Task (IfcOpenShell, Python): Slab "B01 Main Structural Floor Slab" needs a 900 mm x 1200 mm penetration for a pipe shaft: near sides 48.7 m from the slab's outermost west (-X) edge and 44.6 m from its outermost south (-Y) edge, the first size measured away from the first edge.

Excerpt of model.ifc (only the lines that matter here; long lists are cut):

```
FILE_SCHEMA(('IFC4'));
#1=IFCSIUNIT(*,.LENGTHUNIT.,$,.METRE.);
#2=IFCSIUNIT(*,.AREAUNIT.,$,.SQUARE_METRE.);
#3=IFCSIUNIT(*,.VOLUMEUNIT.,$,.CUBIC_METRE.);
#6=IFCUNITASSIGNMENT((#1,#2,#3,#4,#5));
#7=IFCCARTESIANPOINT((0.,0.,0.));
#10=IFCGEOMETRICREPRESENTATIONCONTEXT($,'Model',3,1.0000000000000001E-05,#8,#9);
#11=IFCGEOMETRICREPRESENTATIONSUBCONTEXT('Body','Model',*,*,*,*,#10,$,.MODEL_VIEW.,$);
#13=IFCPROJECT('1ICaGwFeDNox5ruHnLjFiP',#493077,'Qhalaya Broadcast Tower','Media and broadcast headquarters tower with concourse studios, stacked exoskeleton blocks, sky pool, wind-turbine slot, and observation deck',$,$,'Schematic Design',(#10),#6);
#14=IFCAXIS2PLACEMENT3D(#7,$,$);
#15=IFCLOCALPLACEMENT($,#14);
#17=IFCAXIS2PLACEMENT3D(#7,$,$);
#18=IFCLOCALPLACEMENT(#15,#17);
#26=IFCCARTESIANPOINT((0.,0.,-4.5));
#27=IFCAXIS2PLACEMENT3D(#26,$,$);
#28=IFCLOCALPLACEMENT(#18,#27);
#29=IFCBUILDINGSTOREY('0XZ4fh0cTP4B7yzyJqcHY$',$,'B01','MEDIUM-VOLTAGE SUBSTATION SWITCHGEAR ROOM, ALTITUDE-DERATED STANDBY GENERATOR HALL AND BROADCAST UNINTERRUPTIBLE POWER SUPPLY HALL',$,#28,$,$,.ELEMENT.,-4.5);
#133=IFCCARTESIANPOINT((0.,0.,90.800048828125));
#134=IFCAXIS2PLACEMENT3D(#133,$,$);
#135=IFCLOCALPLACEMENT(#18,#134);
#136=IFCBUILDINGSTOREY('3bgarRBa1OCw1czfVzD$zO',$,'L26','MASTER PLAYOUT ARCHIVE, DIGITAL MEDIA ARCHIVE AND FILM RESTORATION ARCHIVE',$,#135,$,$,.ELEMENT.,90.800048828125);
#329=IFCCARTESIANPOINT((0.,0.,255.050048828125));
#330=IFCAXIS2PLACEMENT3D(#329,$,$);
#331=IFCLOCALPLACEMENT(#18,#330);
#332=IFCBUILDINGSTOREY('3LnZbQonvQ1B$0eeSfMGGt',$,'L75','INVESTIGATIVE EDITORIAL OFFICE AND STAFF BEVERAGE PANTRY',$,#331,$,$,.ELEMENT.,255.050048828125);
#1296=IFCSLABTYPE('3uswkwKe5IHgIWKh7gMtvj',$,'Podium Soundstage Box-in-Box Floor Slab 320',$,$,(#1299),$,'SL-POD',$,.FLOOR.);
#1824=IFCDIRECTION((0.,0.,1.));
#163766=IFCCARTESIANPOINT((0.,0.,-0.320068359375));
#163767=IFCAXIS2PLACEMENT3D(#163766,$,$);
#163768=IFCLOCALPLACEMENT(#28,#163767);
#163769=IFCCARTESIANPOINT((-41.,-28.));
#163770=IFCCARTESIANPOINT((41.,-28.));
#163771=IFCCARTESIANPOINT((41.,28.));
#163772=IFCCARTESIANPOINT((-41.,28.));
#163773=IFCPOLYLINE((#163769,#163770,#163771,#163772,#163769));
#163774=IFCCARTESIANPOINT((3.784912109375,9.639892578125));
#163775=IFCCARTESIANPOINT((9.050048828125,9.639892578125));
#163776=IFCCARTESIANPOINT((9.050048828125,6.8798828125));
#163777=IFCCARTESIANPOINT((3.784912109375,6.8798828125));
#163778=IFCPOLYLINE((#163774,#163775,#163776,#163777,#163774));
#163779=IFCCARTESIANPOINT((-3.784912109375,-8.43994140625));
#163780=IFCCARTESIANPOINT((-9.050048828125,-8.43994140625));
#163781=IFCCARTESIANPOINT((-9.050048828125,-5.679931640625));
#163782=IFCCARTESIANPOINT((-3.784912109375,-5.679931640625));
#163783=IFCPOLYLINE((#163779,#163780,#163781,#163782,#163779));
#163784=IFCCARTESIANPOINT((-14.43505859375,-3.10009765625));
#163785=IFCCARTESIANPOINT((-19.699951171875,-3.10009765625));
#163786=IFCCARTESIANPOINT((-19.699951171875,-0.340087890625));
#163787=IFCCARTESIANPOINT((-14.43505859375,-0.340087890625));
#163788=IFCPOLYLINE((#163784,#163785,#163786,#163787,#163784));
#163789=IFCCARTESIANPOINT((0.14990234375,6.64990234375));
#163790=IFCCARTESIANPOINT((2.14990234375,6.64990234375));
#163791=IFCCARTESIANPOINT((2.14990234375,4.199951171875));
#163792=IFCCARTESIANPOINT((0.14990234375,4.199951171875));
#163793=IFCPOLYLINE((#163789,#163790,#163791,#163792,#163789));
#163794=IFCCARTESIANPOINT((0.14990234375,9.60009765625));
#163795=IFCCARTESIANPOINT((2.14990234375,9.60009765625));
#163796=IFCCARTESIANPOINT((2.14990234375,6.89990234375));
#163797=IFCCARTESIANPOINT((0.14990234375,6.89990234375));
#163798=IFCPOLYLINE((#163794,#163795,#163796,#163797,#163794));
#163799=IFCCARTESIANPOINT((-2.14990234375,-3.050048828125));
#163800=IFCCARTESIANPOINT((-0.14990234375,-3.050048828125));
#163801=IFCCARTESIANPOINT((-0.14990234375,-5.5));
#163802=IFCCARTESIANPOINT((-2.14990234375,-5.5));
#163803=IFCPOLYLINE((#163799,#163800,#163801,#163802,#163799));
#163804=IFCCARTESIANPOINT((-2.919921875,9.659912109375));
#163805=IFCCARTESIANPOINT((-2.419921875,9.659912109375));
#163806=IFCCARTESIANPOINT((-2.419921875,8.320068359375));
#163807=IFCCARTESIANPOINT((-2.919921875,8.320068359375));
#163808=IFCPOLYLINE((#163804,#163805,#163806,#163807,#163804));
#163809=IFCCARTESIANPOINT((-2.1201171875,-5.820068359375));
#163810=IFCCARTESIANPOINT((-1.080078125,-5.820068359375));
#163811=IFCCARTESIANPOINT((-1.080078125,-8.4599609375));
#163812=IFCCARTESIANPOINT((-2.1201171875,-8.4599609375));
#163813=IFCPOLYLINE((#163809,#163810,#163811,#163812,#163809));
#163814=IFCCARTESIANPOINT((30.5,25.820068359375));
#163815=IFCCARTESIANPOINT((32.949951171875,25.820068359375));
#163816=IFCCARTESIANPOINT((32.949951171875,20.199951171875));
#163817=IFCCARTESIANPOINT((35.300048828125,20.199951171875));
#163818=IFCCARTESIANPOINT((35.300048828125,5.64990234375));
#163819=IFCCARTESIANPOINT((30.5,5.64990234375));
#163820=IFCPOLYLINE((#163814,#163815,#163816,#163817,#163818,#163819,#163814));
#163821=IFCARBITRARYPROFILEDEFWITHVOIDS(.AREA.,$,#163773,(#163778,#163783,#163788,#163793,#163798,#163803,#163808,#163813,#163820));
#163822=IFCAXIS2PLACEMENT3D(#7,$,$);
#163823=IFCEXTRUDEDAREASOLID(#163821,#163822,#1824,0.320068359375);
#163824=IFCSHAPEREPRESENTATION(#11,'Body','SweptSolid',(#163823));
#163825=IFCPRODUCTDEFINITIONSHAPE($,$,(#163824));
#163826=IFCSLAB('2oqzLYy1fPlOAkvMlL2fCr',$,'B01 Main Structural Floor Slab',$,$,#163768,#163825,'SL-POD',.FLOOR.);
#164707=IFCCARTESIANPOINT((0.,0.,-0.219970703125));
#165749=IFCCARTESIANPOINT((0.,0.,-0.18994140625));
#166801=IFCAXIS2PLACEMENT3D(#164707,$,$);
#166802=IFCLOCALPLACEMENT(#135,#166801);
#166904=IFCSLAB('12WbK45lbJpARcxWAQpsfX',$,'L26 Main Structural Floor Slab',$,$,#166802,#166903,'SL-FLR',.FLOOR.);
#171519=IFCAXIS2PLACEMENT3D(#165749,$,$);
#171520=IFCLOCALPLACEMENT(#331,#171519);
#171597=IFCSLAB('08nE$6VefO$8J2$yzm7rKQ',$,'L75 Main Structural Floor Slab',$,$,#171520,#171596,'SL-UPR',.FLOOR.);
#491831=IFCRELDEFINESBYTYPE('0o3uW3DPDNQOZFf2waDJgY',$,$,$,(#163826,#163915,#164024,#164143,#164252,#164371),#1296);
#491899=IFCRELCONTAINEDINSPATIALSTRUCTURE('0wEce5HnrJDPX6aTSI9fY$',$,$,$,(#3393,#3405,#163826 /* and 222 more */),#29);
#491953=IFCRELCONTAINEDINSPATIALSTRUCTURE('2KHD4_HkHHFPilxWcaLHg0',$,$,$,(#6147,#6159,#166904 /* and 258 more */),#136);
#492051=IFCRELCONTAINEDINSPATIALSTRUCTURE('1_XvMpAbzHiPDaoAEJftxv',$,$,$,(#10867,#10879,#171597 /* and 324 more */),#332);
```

```python
import numpy as np
import ifcopenshell
import ifcopenshell.api.feature
import ifcopenshell.api.geometry
import ifcopenshell.api.root
import ifcopenshell.geom
import ifcopenshell.util.placement
import ifcopenshell.util.representation
import ifcopenshell.util.shape
import ifcopenshell.util.unit

model = ifcopenshell.open("model.ifc")
unit_scale = ifcopenshell.util.unit.calculate_unit_scale(model)
settings = ifcopenshell.geom.settings()


def volume(element):
    """Net volume in cubic metres, openings subtracted."""
    shape = ifcopenshell.geom.create_shape(settings, element)
    return ifcopenshell.util.shape.get_volume(shape.geometry)


slab = model.by_id(163826)
before = volume(slab)

# Extent in the slab's own axes, in metres. The edges named are its -X and -Y sides.
slab_shape = ifcopenshell.geom.create_shape(settings, slab)
vertices = ifcopenshell.util.shape.get_vertices(slab_shape.geometry)
x_min, y_min, bottom = vertices.min(axis=0)
top = vertices[:, 2].max()

opening = ifcopenshell.api.root.create_entity(model, ifc_class="IfcOpeningElement", name="Pipe shaft opening", predefined_type="OPENING")
context = ifcopenshell.util.representation.get_context(model, "Model", "Body", "MODEL_VIEW")
width, depth = 0.9, 1.2
outline = [(0.0, 0.0), (width, 0.0), (width, depth), (0.0, depth), (0.0, 0.0)]
# Overshoot both faces by 50 mm so the cut is clean.
shape = ifcopenshell.api.geometry.add_slab_representation(
    model, context=context, depth=top - bottom + 0.1, polyline=outline
)
ifcopenshell.api.geometry.assign_representation(model, product=opening, representation=shape)

matrix = ifcopenshell.util.placement.get_local_placement(slab.ObjectPlacement)
matrix[:, 3] = matrix @ np.append(np.array([x_min + 48.7, y_min + 44.6, bottom - 0.05]) / unit_scale, 1.0)
ifcopenshell.api.geometry.edit_object_placement(model, product=opening, matrix=matrix, is_si=False)
ifcopenshell.api.feature.add_feature(model, feature=opening, element=slab)

after = volume(slab)

print(f"slab volume {before:.3f} -> {after:.3f} m3")

model.write("model_updated.ifc")
```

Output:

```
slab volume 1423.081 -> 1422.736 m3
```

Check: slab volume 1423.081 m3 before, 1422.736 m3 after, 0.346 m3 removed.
